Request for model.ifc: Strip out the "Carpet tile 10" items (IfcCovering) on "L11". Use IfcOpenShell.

First a look at what the model holds.

```python
import ifcopenshell
import ifcopenshell.util.element

model = ifcopenshell.open("model.ifc")
print(model.schema)
storey = next(s for s in model.by_type("IfcBuildingStorey") if s.Name == "L11")
coverings = [e for e in ifcopenshell.util.element.get_decomposition(storey) if e.is_a("IfcCovering")]
seen = {}
for e in coverings:
    element_type = ifcopenshell.util.element.get_type(e)
    name = element_type.Name if element_type not in (None, e) else None
    seen[name] = seen.get(name, 0) + 1
for name, count in sorted(seen.items(), key=str):
    print(count, "x", name)
```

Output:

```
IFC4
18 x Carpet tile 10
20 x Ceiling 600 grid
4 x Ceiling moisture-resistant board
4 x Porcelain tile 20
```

```python
import ifcopenshell
import ifcopenshell.api.root
import ifcopenshell.util.element

model = ifcopenshell.open("model.ifc")

storey = next(s for s in model.by_type("IfcBuildingStorey") if s.Name == "L11")
coverings = [e for e in ifcopenshell.util.element.get_decomposition(storey) if e.is_a("IfcCovering")]
targets = [e for e in coverings if (t := ifcopenshell.util.element.get_type(e)) not in (None, e) and t.Name == "Carpet tile 10"]

for e in targets:
    ifcopenshell.api.root.remove_product(model, product=e)
print(len(targets), "removed")

model.write("model_edited.ifc")
```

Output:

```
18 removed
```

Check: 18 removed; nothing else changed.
